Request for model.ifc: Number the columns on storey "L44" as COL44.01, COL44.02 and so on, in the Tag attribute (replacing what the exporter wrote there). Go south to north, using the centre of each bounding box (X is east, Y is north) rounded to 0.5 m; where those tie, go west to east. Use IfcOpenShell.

First a look at what the model holds.

```python
import ifcopenshell
import ifcopenshell.util.element
import ifcopenshell.util.placement

model = ifcopenshell.open("model.ifc")
print(model.schema)
storey = next(s for s in model.by_type("IfcBuildingStorey") if s.Name == "L44")
columns = [e for e in ifcopenshell.util.element.get_decomposition(storey) if e.is_a("IfcColumn")]
for e in sorted(columns, key=lambda e: e.id()):
    origin = ifcopenshell.util.placement.get_local_placement(e.ObjectPlacement)[:3, 3]
    print(e.id(), e.Tag, e.Name, origin.round(2) + 0.0, sep=" | ")
```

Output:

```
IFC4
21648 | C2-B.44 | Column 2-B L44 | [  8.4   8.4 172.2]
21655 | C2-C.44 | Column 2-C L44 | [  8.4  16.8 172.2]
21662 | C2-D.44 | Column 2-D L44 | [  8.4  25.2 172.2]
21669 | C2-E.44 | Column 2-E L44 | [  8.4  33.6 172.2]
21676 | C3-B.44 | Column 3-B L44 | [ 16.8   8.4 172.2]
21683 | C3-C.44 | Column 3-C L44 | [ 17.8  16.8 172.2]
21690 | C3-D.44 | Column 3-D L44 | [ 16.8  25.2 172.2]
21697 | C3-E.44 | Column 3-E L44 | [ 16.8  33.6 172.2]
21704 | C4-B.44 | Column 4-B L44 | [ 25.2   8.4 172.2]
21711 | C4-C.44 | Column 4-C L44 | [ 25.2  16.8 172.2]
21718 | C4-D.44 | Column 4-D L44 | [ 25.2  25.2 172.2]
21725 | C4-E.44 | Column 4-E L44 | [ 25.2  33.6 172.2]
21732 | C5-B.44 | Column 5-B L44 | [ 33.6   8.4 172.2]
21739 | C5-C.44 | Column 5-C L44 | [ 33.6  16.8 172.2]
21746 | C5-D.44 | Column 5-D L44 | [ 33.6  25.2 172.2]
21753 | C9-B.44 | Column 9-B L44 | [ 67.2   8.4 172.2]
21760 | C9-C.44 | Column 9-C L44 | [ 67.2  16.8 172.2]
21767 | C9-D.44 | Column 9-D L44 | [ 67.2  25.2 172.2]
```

```python
import ifcopenshell
import ifcopenshell.geom
import ifcopenshell.util.element
import ifcopenshell.util.shape

model = ifcopenshell.open("model.ifc")
settings = ifcopenshell.geom.settings()
settings.set("use-world-coords", True)


def centre(element):
    shape = ifcopenshell.geom.create_shape(settings, element)
    return ifcopenshell.util.shape.get_bbox_centroid(shape.geometry)


storey = next(s for s in model.by_type("IfcBuildingStorey") if s.Name == "L44")
columns = [e for e in ifcopenshell.util.element.get_decomposition(storey) if e.is_a("IfcColumn")]

# Insertion points can sit at a corner or the storey origin, so sort by the geometry (in metres).
centres = {e: centre(e) for e in columns}
columns.sort(key=lambda e: (round(centres[e][1] / 0.5), centres[e][0]))

for i, e in enumerate(columns, start=1):
    number = f"COL44.{i:02d}"
    e.Tag = number
    print(e.id(), number)

model.write("model_rev.ifc")
```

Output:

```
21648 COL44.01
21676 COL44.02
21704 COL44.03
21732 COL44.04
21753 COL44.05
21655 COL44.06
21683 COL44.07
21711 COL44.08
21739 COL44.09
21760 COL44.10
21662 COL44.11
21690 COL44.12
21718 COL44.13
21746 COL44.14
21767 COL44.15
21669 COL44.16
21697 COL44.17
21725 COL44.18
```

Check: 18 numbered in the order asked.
